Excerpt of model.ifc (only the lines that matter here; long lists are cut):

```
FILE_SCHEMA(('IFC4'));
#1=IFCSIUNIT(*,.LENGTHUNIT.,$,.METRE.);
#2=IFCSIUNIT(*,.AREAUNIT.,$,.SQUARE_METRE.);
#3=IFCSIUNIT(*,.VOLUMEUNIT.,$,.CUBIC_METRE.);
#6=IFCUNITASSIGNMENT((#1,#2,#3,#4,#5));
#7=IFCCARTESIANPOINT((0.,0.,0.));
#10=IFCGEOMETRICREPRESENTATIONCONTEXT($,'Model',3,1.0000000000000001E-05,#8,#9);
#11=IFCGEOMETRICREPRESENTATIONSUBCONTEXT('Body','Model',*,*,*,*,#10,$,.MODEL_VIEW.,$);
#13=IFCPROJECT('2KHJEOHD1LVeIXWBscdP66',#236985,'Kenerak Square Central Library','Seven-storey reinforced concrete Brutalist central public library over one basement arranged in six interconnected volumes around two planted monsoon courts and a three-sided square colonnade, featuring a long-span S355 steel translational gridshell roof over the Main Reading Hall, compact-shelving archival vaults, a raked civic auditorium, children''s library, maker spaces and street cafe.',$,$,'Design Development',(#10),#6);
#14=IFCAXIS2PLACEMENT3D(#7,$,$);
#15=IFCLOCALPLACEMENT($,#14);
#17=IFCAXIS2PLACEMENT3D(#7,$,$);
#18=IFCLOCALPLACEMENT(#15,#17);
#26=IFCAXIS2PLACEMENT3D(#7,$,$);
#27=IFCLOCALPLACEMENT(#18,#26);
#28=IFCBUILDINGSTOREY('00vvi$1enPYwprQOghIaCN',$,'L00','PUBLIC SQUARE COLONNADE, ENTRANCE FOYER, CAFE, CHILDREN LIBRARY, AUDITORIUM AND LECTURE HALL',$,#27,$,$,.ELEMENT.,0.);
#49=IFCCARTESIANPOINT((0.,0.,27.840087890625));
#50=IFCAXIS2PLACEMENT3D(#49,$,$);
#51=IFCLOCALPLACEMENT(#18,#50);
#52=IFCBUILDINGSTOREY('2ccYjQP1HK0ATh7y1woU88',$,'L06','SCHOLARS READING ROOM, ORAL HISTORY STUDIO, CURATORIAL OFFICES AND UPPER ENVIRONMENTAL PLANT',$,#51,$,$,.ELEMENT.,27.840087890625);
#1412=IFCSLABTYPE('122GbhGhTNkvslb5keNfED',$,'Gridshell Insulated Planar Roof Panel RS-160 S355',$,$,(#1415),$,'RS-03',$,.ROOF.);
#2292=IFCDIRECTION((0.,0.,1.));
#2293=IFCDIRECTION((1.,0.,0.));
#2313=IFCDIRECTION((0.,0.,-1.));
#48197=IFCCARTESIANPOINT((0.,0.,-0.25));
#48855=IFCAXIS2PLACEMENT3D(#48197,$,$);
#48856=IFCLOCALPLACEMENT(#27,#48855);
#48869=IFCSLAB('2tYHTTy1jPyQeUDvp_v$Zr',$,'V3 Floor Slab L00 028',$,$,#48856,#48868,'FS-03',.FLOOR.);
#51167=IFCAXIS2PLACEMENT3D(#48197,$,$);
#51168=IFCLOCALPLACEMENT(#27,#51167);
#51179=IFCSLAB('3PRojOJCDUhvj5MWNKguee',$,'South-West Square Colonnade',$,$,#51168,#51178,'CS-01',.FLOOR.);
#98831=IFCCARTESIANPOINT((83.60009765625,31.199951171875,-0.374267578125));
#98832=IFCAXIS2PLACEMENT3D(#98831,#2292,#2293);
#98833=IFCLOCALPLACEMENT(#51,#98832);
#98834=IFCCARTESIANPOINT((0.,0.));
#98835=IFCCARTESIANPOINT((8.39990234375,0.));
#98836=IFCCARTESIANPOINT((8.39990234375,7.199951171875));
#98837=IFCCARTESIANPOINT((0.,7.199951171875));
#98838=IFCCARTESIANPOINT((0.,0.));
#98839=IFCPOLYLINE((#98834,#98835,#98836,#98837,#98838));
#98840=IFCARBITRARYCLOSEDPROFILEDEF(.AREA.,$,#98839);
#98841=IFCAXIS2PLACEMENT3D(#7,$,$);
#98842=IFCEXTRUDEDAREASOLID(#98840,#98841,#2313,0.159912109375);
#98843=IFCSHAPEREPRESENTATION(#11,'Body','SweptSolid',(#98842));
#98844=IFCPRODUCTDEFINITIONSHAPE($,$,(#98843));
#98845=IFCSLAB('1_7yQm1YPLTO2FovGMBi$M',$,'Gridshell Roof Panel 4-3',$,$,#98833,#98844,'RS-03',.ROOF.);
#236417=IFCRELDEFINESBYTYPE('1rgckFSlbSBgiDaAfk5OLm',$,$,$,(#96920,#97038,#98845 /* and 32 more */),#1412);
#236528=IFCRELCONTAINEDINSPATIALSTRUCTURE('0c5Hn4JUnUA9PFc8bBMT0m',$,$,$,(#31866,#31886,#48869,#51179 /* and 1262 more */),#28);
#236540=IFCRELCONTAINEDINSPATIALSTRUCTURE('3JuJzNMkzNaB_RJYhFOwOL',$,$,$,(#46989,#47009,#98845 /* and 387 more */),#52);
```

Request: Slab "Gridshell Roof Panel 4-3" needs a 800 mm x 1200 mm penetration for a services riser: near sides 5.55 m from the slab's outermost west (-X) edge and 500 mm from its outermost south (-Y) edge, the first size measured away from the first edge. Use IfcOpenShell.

```python
import numpy as np
import ifcopenshell
import ifcopenshell.api.feature
import ifcopenshell.api.geometry
import ifcopenshell.api.root
import ifcopenshell.geom
import ifcopenshell.util.placement
import ifcopenshell.util.representation
import ifcopenshell.util.shape
import ifcopenshell.util.unit

model = ifcopenshell.open("model.ifc")
unit_scale = ifcopenshell.util.unit.calculate_unit_scale(model)
settings = ifcopenshell.geom.settings()


def volume(element):
    """Net volume in cubic metres, openings subtracted."""
    shape = ifcopenshell.geom.create_shape(settings, element)
    return ifcopenshell.util.shape.get_volume(shape.geometry)


slab = model.by_guid("1_7yQm1YPLTO2FovGMBi$M")
before = volume(slab)

# Extent in the slab's own axes, in metres. The edges named are its -X and -Y sides.
slab_shape = ifcopenshell.geom.create_shape(settings, slab)
vertices = ifcopenshell.util.shape.get_vertices(slab_shape.geometry)
x_min, y_min, bottom = vertices.min(axis=0)
top = vertices[:, 2].max()

opening = ifcopenshell.api.root.create_entity(model, ifc_class="IfcOpeningElement", name="Services riser opening", predefined_type="OPENING")
context = ifcopenshell.util.representation.get_context(model, "Model", "Body", "MODEL_VIEW")
width, depth = 0.8, 1.2
outline = [(0.0, 0.0), (width, 0.0), (width, depth), (0.0, depth), (0.0, 0.0)]
# Overshoot both faces by 50 mm so the cut is clean.
shape = ifcopenshell.api.geometry.add_slab_representation(
    model, context=context, depth=top - bottom + 0.1, polyline=outline
)
ifcopenshell.api.geometry.assign_representation(model, product=opening, representation=shape)

matrix = ifcopenshell.util.placement.get_local_placement(slab.ObjectPlacement)
matrix[:, 3] = matrix @ np.append(np.array([x_min + 5.55, y_min + 0.5, bottom - 0.05]) / unit_scale, 1.0)
ifcopenshell.api.geometry.edit_object_placement(model, product=opening, matrix=matrix, is_si=False)
ifcopenshell.api.feature.add_feature(model, feature=opening, element=slab)

after = volume(slab)

print(f"slab volume {before:.3f} -> {after:.3f} m3")

model.write("model_rev.ifc")
```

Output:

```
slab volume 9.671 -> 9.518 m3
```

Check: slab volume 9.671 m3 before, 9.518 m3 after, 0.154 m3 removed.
